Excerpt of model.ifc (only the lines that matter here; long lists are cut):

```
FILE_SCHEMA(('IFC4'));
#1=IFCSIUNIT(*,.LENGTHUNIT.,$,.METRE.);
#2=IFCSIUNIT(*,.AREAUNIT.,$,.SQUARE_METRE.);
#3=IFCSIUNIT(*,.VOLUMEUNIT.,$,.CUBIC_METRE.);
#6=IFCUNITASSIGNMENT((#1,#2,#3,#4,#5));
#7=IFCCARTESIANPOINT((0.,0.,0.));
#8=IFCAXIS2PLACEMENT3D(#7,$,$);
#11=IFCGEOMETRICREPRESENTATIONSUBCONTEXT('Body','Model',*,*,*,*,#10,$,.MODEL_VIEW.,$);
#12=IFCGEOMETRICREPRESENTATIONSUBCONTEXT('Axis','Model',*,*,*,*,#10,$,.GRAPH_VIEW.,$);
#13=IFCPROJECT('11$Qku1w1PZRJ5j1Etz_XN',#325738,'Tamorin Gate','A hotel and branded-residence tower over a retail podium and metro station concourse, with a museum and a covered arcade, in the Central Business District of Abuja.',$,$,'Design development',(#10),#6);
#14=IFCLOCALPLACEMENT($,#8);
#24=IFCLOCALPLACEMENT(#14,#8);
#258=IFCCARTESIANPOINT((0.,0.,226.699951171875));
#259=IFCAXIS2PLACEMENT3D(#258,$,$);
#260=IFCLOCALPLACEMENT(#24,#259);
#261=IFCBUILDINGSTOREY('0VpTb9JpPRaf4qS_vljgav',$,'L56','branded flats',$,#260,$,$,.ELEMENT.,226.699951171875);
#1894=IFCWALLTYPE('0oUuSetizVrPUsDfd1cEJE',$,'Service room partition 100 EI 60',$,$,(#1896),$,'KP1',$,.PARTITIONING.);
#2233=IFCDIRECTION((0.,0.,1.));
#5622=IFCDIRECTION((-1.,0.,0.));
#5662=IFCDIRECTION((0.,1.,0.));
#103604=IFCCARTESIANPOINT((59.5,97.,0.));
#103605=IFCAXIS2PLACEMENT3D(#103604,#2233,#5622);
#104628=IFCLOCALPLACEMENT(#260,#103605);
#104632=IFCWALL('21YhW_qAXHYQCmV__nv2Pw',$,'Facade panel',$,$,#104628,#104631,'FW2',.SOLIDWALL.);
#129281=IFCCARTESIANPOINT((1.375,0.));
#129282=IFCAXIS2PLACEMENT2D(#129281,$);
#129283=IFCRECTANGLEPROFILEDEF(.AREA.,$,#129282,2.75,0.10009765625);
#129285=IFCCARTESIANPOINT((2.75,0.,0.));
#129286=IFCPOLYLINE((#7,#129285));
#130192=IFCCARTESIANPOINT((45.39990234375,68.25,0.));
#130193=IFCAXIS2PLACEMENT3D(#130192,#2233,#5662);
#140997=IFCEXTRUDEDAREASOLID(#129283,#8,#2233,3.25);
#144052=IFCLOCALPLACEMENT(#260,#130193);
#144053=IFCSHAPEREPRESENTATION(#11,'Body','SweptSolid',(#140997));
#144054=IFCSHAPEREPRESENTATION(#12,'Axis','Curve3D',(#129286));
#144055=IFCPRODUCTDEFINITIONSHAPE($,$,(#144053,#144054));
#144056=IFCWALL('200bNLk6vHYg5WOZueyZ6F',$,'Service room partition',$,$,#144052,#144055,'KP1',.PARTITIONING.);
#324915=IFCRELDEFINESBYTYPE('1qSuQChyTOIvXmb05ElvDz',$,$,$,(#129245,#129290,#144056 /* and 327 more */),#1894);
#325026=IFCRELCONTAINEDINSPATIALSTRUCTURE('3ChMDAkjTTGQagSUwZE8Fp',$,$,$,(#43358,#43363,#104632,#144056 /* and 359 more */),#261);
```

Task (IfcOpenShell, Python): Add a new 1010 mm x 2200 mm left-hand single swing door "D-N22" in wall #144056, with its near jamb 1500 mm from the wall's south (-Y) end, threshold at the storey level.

```python
import numpy as np
import ifcopenshell
import ifcopenshell.api.feature
import ifcopenshell.api.geometry
import ifcopenshell.api.root
import ifcopenshell.api.spatial
import ifcopenshell.geom
import ifcopenshell.util.element
import ifcopenshell.util.placement
import ifcopenshell.util.representation
import ifcopenshell.util.shape
import ifcopenshell.util.unit

model = ifcopenshell.open("model.ifc")
unit_scale = ifcopenshell.util.unit.calculate_unit_scale(model)
settings = ifcopenshell.geom.settings()


def volume(element):
    """Net volume in cubic metres, openings subtracted."""
    shape = ifcopenshell.geom.create_shape(settings, element)
    return ifcopenshell.util.shape.get_volume(shape.geometry)


wall = model.by_guid("200bNLk6vHYg5WOZueyZ6F")
storey = ifcopenshell.util.element.get_container(wall, ifc_class="IfcBuildingStorey")
context = ifcopenshell.util.representation.get_context(model, "Model", "Body", "MODEL_VIEW")
before = volume(wall)

width, height, from_end, sill = 1.01, 2.2, 1.5, 0.0  # metres

# The wall runs along its own X axis, and the end named is its -X end.
wall_shape = ifcopenshell.geom.create_shape(settings, wall)
x, y, z = ifcopenshell.util.shape.get_vertices(wall_shape.geometry).T
start = x.min() + from_end
face, thickness = float(y.min()), float(y.max() - y.min())
wall_matrix = ifcopenshell.util.placement.get_local_placement(wall.ObjectPlacement)
level = ifcopenshell.util.placement.get_local_placement(storey.ObjectPlacement)[2, 3]


def in_wall(x, y):
    """Placement at x, y metres in the wall's axes, at sill height."""
    matrix = wall_matrix.copy()
    matrix[:, 3] = wall_matrix @ np.array([x / unit_scale, y / unit_scale, 0.0, 1.0])
    matrix[2, 3] = level + sill / unit_scale
    return matrix


# Opening: a box that overshoots both wall faces by 50 mm.
opening = ifcopenshell.api.root.create_entity(model, ifc_class="IfcOpeningElement", predefined_type="OPENING")
box = ifcopenshell.api.geometry.add_wall_representation(
    model, context=context, length=width, height=height, thickness=thickness + 0.1
)
ifcopenshell.api.geometry.assign_representation(model, product=opening, representation=box)
ifcopenshell.api.geometry.edit_object_placement(model, product=opening, matrix=in_wall(start, face - 0.05), is_si=False)
ifcopenshell.api.feature.add_feature(model, feature=opening, element=wall)

door = ifcopenshell.api.root.create_entity(model, ifc_class="IfcDoor", name="D-N22", predefined_type="DOOR")
door.OverallWidth, door.OverallHeight = width / unit_scale, height / unit_scale
door.OperationType = "SINGLE_SWING_LEFT"
body = ifcopenshell.api.geometry.add_door_representation(
    model,
    context=context,
    overall_width=door.OverallWidth,
    overall_height=door.OverallHeight,
    operation_type="SINGLE_SWING_LEFT",
    lining_properties={"LiningDepth": thickness / unit_scale, "ThresholdDepth": thickness / unit_scale},
)
ifcopenshell.api.geometry.assign_representation(model, product=door, representation=body)
ifcopenshell.api.spatial.assign_container(model, products=[door], relating_structure=storey)
ifcopenshell.api.feature.add_filling(model, opening=opening, element=door)

# The lining spans the wall, so the door starts at the wall face.
ifcopenshell.api.geometry.edit_object_placement(model, product=door, matrix=in_wall(start, face), is_si=False)

after = volume(wall)

print(f"wall volume {before:.3f} -> {after:.3f} m3")

model.write("model_v2.ifc")
```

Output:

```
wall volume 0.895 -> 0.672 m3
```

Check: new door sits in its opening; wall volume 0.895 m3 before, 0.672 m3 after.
